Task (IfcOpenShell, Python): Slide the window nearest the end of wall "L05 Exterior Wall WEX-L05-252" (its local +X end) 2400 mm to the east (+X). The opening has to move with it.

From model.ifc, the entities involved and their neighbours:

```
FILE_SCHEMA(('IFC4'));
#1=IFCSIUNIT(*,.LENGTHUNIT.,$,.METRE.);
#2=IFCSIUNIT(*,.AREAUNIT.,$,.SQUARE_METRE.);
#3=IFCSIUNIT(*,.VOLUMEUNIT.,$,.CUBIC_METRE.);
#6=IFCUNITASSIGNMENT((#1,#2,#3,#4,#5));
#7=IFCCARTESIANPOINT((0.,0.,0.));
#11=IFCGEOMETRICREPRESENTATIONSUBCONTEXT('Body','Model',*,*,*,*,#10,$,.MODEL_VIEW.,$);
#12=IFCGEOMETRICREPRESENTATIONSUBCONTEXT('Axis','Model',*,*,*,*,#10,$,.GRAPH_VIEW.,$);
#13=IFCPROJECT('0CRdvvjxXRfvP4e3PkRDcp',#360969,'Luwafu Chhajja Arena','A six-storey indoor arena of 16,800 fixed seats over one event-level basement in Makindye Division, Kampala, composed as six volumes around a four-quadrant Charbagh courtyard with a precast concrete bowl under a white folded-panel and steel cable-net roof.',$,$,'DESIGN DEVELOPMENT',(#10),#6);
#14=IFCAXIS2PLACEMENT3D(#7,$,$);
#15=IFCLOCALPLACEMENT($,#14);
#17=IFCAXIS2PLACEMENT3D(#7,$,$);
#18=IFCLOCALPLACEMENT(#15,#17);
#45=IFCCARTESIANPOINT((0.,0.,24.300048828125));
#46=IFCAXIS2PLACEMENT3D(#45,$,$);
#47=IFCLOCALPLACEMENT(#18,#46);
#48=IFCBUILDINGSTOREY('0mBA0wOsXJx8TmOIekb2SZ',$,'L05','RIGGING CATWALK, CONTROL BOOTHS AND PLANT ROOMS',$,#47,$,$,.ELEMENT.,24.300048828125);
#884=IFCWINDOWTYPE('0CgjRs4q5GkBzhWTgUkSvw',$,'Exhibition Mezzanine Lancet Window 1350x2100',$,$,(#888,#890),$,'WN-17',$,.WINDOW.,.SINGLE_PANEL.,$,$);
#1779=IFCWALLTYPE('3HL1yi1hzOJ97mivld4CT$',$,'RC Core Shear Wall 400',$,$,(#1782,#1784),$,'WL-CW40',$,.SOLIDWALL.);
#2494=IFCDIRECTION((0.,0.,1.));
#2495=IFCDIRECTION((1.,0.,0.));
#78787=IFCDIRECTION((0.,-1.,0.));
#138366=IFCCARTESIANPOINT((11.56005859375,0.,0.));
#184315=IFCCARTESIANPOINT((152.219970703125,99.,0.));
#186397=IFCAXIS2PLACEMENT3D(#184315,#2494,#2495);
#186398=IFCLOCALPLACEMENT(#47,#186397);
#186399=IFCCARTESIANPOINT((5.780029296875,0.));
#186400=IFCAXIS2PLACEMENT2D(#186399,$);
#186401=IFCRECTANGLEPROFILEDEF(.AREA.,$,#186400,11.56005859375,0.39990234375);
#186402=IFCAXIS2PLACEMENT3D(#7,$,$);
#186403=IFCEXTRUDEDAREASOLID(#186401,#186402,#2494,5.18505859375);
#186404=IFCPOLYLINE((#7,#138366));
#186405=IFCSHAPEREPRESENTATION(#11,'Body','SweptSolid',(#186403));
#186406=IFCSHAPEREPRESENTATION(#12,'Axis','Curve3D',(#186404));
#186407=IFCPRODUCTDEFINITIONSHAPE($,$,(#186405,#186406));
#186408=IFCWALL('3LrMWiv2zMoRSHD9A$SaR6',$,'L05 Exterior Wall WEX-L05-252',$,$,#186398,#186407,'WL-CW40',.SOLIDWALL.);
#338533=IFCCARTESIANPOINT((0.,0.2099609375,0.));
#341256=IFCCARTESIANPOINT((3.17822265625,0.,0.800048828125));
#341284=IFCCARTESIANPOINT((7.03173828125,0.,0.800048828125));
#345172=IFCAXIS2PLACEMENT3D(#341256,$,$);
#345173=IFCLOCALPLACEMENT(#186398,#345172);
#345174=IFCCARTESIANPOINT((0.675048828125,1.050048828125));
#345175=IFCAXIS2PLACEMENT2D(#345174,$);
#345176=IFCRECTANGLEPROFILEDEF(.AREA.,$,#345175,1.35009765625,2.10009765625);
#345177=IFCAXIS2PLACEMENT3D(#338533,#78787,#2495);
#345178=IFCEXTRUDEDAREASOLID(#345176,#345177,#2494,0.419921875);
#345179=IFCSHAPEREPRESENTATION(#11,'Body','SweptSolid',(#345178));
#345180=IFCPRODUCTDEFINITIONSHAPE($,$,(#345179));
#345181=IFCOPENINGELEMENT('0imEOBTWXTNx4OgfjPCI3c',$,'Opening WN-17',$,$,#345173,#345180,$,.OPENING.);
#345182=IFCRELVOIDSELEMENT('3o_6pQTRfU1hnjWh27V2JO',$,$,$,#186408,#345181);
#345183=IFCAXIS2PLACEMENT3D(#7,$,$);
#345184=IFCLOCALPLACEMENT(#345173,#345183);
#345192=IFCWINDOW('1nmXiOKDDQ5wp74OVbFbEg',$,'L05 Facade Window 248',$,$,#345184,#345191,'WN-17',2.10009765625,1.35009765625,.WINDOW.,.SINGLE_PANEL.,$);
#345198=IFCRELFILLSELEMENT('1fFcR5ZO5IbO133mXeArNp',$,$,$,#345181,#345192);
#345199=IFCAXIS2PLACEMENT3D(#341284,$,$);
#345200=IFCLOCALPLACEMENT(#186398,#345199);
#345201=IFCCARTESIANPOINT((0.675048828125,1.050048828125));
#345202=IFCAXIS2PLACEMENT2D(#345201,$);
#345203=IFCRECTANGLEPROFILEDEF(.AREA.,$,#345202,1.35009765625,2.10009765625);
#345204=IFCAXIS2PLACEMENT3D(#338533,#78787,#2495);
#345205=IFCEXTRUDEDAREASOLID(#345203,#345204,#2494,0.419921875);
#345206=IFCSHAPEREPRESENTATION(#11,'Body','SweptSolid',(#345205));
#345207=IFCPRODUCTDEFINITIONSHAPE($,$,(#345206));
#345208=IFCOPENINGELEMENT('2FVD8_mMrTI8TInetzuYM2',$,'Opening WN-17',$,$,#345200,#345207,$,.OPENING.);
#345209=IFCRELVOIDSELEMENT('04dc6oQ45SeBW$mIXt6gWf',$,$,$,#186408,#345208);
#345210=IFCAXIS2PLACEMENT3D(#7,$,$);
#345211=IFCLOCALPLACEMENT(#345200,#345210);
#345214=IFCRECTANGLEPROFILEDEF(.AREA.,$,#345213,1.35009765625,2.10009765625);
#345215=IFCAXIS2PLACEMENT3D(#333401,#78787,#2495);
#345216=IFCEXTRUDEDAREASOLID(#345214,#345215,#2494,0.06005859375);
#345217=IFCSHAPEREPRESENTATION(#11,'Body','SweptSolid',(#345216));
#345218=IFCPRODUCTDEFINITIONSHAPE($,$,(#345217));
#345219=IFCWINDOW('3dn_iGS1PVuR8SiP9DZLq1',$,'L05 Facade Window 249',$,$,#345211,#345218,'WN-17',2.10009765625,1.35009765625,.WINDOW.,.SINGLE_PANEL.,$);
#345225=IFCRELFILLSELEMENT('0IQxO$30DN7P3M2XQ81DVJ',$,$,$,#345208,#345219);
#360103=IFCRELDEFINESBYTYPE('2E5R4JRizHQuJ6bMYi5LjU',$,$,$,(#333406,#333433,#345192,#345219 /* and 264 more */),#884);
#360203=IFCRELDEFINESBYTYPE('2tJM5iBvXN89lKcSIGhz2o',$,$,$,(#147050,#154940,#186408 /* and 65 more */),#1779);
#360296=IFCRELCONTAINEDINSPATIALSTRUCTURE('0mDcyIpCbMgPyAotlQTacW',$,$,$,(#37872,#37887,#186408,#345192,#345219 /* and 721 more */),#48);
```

```python
import ifcopenshell
import ifcopenshell.api.geometry
import ifcopenshell.util.placement

model = ifcopenshell.open("model.ifc")

window = model.by_guid("3dn_iGS1PVuR8SiP9DZLq1")
opening = window.FillsVoids[0].RelatingOpeningElement
wall = opening.VoidsElements[0].RelatingBuildingElement

wall_matrix = ifcopenshell.util.placement.get_local_placement(wall.ObjectPlacement)
shift = wall_matrix[:3, 0] * 2.4
before = ifcopenshell.util.placement.get_local_placement(window.ObjectPlacement)[:3, 3].copy()

# The window is placed relative to its opening, so it follows when the opening moves.
matrix = ifcopenshell.util.placement.get_local_placement(opening.ObjectPlacement)
matrix[:3, 3] += shift
ifcopenshell.api.geometry.edit_object_placement(
    model, product=opening, matrix=matrix, is_si=False, should_transform_children=True
)

after = ifcopenshell.util.placement.get_local_placement(window.ObjectPlacement)[:3, 3]
print("window moved by", (after - before).round(3) + 0.0)

model.write("model_updated.ifc")
```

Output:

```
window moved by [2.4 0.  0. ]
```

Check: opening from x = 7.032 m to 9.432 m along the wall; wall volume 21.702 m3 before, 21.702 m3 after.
